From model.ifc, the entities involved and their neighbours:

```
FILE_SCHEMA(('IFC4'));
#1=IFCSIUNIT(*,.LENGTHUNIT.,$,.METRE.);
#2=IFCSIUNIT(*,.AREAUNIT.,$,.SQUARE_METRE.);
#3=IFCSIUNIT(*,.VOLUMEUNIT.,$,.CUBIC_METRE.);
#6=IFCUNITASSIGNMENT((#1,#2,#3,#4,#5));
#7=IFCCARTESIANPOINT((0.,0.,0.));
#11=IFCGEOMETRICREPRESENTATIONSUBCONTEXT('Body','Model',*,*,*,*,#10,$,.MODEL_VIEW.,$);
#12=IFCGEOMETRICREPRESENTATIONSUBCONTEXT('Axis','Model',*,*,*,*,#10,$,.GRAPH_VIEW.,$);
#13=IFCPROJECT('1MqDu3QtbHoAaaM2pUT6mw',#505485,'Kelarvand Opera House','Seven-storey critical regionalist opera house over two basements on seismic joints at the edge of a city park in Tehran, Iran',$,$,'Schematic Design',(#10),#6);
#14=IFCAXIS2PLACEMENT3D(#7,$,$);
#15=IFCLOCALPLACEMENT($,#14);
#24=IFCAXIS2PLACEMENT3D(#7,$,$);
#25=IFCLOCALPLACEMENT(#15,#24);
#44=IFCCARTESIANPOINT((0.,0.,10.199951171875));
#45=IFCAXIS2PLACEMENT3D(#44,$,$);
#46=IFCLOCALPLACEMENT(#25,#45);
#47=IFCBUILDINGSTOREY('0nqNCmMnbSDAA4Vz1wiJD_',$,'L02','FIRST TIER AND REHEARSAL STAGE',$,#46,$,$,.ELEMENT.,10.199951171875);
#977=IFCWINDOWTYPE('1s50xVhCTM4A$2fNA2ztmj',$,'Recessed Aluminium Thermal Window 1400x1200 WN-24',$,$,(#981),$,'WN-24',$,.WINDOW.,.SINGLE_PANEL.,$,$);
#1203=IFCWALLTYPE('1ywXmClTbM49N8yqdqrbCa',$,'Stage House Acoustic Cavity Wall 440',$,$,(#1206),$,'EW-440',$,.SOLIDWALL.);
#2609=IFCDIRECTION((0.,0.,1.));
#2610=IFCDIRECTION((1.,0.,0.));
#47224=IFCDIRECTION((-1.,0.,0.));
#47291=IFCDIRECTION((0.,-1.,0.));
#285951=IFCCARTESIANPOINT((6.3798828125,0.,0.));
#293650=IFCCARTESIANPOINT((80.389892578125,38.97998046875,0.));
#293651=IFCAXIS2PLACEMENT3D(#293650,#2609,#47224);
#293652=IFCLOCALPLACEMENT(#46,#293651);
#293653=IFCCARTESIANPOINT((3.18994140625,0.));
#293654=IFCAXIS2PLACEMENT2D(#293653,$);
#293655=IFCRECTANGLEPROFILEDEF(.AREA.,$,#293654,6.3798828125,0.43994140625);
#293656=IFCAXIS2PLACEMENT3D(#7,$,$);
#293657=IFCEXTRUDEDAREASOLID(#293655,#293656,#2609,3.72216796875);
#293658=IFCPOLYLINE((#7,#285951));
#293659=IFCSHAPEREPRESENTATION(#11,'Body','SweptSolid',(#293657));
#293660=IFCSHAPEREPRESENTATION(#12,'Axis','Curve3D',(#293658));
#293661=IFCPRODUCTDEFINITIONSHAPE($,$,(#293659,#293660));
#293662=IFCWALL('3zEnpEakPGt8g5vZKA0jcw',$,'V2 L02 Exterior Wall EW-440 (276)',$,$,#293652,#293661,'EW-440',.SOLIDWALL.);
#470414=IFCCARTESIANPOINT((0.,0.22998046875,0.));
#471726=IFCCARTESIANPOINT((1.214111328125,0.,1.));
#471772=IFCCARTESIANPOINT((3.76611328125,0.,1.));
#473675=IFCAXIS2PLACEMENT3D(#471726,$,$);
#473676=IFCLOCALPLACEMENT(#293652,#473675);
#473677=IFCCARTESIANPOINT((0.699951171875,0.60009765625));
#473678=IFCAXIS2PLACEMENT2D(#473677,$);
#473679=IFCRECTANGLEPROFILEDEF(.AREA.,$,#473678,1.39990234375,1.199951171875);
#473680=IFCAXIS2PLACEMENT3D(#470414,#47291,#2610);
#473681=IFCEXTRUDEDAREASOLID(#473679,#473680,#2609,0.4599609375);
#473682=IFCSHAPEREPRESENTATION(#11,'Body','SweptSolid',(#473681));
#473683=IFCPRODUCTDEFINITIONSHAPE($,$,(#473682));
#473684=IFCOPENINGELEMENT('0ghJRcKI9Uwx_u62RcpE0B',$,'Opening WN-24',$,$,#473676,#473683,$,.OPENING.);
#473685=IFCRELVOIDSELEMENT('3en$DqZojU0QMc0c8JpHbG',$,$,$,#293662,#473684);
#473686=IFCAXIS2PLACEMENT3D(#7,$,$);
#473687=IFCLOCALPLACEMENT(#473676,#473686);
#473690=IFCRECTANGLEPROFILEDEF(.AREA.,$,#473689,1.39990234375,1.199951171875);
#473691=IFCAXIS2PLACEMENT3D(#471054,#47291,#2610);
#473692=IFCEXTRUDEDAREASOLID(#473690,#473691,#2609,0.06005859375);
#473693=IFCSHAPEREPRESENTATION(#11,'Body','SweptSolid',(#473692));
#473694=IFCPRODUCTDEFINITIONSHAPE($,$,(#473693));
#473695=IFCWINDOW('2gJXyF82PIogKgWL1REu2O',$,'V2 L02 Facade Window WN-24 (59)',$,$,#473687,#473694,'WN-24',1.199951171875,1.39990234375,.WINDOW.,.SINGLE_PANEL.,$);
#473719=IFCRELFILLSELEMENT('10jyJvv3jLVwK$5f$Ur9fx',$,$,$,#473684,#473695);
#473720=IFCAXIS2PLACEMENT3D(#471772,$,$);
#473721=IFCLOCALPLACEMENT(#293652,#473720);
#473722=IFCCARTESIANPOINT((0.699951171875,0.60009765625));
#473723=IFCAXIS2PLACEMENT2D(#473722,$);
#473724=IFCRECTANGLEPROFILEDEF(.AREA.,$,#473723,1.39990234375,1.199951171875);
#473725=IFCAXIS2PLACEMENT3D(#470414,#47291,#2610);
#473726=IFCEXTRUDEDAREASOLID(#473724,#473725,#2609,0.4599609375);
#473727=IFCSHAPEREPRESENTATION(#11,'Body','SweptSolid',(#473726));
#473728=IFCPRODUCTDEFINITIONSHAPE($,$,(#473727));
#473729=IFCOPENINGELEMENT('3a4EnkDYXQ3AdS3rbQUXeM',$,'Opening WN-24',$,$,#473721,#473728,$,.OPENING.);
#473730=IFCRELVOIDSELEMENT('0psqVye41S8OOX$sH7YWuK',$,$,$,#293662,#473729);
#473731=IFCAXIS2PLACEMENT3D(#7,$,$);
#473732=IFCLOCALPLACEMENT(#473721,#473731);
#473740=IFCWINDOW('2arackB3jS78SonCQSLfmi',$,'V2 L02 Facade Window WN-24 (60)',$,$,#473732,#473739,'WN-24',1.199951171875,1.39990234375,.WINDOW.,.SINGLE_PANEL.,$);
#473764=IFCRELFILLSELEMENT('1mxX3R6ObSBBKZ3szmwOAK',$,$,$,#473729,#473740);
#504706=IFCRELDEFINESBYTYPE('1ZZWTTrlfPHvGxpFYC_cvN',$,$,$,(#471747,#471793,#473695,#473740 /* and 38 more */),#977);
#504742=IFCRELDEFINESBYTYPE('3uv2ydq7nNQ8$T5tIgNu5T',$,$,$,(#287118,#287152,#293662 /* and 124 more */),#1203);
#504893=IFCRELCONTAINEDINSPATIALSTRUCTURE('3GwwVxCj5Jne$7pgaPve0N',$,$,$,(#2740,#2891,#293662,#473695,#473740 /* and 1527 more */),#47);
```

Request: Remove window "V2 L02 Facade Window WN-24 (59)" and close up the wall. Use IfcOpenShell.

```python
import ifcopenshell
import ifcopenshell.api.feature
import ifcopenshell.api.root
import ifcopenshell.geom
import ifcopenshell.util.shape

model = ifcopenshell.open("model.ifc")
settings = ifcopenshell.geom.settings()


def volume(element):
    """Net volume in cubic metres, openings subtracted."""
    shape = ifcopenshell.geom.create_shape(settings, element)
    return ifcopenshell.util.shape.get_volume(shape.geometry)


window = model.by_guid("2gJXyF82PIogKgWL1REu2O")
opening = window.FillsVoids[0].RelatingOpeningElement
wall = opening.VoidsElements[0].RelatingBuildingElement
before = volume(wall)

ifcopenshell.api.root.remove_product(model, product=window)
ifcopenshell.api.feature.remove_feature(model, feature=opening)

after = volume(wall)

print(f"wall volume {before:.3f} -> {after:.3f} m3")

model.write("model-out.ifc")
```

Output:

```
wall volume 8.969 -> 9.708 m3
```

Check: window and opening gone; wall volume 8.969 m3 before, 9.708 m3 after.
